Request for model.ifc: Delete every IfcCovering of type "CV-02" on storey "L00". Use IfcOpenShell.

First a look at what the model holds.

```python
import ifcopenshell
import ifcopenshell.util.element

model = ifcopenshell.open("model.ifc")
print(model.schema)
storey = next(s for s in model.by_type("IfcBuildingStorey") if s.Name == "L00")
coverings = [e for e in ifcopenshell.util.element.get_decomposition(storey) if e.is_a("IfcCovering")]
seen = {}
for e in coverings:
    element_type = ifcopenshell.util.element.get_type(e)
    name = element_type.Name if element_type not in (None, e) else None
    seen[name] = seen.get(name, 0) + 1
for name, count in sorted(seen.items(), key=str):
    print(count, "x", name)
```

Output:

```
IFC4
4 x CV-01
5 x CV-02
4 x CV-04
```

```python
import ifcopenshell
import ifcopenshell.api.root
import ifcopenshell.util.element

model = ifcopenshell.open("model.ifc")

storey = next(s for s in model.by_type("IfcBuildingStorey") if s.Name == "L00")
coverings = [e for e in ifcopenshell.util.element.get_decomposition(storey) if e.is_a("IfcCovering")]
targets = [e for e in coverings if (t := ifcopenshell.util.element.get_type(e)) not in (None, e) and t.Name == "CV-02"]

for e in targets:
    ifcopenshell.api.root.remove_product(model, product=e)
print(len(targets), "removed")

model.write("model-out.ifc")
```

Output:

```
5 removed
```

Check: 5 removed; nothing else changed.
